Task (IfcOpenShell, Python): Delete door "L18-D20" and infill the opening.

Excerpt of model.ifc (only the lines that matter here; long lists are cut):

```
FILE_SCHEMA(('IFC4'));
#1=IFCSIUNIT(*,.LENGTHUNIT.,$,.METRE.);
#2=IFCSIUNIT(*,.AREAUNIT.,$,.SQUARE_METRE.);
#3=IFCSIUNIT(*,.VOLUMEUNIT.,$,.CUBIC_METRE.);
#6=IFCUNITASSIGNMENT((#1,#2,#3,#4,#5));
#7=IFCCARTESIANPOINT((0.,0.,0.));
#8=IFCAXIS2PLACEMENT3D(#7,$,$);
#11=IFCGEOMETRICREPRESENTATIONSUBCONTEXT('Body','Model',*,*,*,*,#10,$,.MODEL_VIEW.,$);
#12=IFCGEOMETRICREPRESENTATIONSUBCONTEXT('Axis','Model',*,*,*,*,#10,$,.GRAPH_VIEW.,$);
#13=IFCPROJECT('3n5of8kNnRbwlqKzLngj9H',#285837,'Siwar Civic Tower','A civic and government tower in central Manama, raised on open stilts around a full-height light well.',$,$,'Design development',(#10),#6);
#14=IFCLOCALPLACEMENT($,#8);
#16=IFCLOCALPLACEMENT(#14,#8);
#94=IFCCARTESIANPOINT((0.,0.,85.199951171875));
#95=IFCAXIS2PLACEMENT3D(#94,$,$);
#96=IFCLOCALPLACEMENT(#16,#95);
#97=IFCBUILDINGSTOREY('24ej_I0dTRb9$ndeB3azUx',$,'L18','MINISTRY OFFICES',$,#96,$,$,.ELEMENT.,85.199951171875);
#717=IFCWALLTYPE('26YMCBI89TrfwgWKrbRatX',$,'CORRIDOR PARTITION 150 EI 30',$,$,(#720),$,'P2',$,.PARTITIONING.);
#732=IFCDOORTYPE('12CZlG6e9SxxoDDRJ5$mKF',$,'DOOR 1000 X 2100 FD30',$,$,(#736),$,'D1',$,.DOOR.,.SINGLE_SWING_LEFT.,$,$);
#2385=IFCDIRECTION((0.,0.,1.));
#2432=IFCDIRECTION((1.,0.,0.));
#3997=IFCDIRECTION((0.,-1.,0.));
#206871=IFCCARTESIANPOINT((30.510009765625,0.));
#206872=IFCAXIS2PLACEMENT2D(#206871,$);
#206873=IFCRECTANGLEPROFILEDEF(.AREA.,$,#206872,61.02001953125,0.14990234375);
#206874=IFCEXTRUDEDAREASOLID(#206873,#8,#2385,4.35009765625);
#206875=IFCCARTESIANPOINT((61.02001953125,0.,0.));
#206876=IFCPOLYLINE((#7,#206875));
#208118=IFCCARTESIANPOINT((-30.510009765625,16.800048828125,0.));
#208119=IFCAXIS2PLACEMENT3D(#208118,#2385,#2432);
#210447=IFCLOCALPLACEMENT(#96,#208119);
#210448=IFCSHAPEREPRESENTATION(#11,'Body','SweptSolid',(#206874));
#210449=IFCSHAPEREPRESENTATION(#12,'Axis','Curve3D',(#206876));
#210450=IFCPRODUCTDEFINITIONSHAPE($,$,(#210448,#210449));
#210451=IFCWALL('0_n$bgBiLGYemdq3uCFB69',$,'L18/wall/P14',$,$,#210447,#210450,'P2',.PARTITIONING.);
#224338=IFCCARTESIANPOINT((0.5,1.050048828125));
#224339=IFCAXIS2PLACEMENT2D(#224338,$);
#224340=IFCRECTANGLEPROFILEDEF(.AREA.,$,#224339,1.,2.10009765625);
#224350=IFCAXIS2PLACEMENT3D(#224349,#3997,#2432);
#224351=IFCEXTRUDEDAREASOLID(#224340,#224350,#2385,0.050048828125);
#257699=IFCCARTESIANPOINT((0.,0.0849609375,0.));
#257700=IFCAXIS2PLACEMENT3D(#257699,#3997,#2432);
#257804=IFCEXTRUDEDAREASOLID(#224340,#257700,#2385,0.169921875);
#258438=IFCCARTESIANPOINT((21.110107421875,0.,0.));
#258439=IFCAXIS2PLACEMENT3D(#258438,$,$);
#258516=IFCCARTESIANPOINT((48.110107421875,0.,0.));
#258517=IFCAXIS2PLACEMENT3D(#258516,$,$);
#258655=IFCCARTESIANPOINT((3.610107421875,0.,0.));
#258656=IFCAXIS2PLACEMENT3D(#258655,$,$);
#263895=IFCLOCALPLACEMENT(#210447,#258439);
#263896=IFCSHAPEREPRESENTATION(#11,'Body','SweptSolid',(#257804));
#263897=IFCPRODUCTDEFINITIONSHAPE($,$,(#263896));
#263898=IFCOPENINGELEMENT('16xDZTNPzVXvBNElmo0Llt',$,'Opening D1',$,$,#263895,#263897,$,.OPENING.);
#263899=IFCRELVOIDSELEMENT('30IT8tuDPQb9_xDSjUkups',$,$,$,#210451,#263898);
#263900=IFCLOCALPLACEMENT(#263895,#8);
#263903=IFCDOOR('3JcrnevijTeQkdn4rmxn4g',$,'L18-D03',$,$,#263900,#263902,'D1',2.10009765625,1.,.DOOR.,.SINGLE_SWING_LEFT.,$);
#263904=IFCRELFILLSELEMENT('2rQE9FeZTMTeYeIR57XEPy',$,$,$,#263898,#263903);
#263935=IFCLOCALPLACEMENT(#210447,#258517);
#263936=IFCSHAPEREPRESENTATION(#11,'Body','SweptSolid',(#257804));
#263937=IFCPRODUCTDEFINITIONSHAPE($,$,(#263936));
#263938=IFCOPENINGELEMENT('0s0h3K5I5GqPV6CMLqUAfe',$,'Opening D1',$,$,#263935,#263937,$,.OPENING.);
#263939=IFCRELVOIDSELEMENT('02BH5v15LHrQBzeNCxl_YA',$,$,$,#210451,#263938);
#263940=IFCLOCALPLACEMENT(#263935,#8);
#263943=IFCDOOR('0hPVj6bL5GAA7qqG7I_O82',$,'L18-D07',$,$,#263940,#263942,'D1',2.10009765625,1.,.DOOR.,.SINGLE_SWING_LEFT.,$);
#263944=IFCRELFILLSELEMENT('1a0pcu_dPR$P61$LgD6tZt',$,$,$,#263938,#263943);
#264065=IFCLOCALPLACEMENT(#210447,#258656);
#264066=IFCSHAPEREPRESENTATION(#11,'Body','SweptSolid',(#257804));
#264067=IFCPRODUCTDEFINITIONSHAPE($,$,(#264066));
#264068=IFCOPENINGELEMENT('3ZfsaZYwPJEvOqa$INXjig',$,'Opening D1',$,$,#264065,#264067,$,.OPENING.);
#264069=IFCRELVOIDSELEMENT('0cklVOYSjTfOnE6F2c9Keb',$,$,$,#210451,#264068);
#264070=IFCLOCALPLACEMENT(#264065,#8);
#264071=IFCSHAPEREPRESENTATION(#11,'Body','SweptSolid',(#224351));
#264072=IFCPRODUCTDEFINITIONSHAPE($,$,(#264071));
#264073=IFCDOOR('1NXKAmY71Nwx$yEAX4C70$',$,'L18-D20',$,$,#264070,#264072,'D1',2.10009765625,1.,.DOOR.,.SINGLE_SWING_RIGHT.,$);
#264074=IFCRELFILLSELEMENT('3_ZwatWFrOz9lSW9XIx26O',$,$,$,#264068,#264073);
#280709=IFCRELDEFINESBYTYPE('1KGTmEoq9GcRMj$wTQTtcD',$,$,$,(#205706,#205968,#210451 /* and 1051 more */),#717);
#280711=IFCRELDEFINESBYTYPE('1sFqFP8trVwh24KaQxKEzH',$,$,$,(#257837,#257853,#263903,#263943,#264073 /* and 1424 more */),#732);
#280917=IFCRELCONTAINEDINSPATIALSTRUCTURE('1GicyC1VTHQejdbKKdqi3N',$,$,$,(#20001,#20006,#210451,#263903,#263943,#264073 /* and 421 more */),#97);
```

```python
import ifcopenshell
import ifcopenshell.api.feature
import ifcopenshell.api.root
import ifcopenshell.geom
import ifcopenshell.util.shape

model = ifcopenshell.open("model.ifc")
settings = ifcopenshell.geom.settings()


def volume(element):
    """Net volume in cubic metres, openings subtracted."""
    shape = ifcopenshell.geom.create_shape(settings, element)
    return ifcopenshell.util.shape.get_volume(shape.geometry)


door = model.by_guid("1NXKAmY71Nwx$yEAX4C70$")
opening = door.FillsVoids[0].RelatingOpeningElement
wall = opening.VoidsElements[0].RelatingBuildingElement
before = volume(wall)

ifcopenshell.api.root.remove_product(model, product=door)
ifcopenshell.api.feature.remove_feature(model, feature=opening)

after = volume(wall)

print(f"wall volume {before:.3f} -> {after:.3f} m3")

model.write("model_v2.ifc")
```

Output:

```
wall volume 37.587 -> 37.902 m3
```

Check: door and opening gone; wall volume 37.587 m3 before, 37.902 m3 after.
